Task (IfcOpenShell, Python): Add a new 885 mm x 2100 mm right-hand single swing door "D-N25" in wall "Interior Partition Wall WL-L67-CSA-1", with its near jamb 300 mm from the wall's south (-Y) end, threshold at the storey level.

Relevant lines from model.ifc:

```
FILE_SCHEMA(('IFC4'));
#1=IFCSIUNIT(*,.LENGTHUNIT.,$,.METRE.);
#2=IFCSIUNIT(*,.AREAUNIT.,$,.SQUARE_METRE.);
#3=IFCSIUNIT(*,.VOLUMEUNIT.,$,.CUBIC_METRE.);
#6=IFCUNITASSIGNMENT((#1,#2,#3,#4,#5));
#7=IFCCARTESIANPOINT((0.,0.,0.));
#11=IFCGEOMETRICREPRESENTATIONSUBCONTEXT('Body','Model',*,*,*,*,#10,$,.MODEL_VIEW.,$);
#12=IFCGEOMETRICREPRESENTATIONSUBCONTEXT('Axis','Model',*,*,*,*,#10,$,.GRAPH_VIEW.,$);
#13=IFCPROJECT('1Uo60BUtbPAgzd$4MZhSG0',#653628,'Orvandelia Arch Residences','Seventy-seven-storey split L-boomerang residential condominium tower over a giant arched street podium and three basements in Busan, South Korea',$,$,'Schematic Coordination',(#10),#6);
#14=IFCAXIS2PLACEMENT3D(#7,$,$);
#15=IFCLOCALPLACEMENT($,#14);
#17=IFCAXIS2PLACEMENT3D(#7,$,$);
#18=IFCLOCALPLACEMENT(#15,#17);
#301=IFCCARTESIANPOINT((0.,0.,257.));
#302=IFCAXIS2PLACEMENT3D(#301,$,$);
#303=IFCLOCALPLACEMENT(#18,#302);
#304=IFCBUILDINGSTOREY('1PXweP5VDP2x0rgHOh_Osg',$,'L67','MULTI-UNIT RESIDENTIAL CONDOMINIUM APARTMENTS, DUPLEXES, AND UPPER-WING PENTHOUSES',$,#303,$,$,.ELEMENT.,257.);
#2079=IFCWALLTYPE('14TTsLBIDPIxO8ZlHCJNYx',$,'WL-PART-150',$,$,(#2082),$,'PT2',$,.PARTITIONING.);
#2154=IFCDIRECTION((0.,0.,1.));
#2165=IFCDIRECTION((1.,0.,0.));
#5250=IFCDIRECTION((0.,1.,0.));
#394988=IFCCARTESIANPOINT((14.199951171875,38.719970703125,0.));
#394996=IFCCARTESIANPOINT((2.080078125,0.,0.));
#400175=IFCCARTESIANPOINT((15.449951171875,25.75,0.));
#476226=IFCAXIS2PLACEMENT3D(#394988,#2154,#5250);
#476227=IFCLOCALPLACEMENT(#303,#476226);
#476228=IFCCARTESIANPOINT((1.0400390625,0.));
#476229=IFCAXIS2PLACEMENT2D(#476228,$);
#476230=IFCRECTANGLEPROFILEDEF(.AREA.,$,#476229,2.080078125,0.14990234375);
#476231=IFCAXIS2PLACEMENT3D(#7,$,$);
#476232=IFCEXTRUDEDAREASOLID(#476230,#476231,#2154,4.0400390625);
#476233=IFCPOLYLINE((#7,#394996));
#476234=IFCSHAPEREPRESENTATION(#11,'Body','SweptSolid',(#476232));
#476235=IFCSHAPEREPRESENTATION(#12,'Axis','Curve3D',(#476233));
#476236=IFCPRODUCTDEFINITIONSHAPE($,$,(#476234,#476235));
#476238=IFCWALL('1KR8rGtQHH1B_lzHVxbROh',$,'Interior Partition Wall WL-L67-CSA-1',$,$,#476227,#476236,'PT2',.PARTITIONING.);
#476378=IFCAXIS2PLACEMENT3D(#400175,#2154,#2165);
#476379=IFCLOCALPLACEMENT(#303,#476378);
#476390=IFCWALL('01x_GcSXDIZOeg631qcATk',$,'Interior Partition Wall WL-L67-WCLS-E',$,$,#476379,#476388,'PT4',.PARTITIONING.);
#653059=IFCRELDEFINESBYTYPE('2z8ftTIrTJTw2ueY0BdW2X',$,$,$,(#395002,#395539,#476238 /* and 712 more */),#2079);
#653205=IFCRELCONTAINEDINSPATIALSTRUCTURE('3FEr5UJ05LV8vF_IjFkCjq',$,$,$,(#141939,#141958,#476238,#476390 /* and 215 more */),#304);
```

```python
import numpy as np
import ifcopenshell
import ifcopenshell.api.feature
import ifcopenshell.api.geometry
import ifcopenshell.api.root
import ifcopenshell.api.spatial
import ifcopenshell.geom
import ifcopenshell.util.element
import ifcopenshell.util.placement
import ifcopenshell.util.representation
import ifcopenshell.util.shape
import ifcopenshell.util.unit

model = ifcopenshell.open("model.ifc")
unit_scale = ifcopenshell.util.unit.calculate_unit_scale(model)
settings = ifcopenshell.geom.settings()


def volume(element):
    """Net volume in cubic metres, openings subtracted."""
    shape = ifcopenshell.geom.create_shape(settings, element)
    return ifcopenshell.util.shape.get_volume(shape.geometry)


wall = model.by_guid("1KR8rGtQHH1B_lzHVxbROh")
storey = ifcopenshell.util.element.get_container(wall, ifc_class="IfcBuildingStorey")
context = ifcopenshell.util.representation.get_context(model, "Model", "Body", "MODEL_VIEW")
before = volume(wall)

width, height, from_end, sill = 0.885, 2.1, 0.3, 0.0  # metres

# The wall runs along its own X axis, and the end named is its -X end.
wall_shape = ifcopenshell.geom.create_shape(settings, wall)
x, y, z = ifcopenshell.util.shape.get_vertices(wall_shape.geometry).T
start = x.min() + from_end
face, thickness = float(y.min()), float(y.max() - y.min())
wall_matrix = ifcopenshell.util.placement.get_local_placement(wall.ObjectPlacement)
level = ifcopenshell.util.placement.get_local_placement(storey.ObjectPlacement)[2, 3]


def in_wall(x, y):
    """Placement at x, y metres in the wall's axes, at sill height."""
    matrix = wall_matrix.copy()
    matrix[:, 3] = wall_matrix @ np.array([x / unit_scale, y / unit_scale, 0.0, 1.0])
    matrix[2, 3] = level + sill / unit_scale
    return matrix


# Opening: a box that overshoots both wall faces by 50 mm.
opening = ifcopenshell.api.root.create_entity(model, ifc_class="IfcOpeningElement", predefined_type="OPENING")
box = ifcopenshell.api.geometry.add_wall_representation(
    model, context=context, length=width, height=height, thickness=thickness + 0.1
)
ifcopenshell.api.geometry.assign_representation(model, product=opening, representation=box)
ifcopenshell.api.geometry.edit_object_placement(model, product=opening, matrix=in_wall(start, face - 0.05), is_si=False)
ifcopenshell.api.feature.add_feature(model, feature=opening, element=wall)

door = ifcopenshell.api.root.create_entity(model, ifc_class="IfcDoor", name="D-N25", predefined_type="DOOR")
door.OverallWidth, door.OverallHeight = width / unit_scale, height / unit_scale
door.OperationType = "SINGLE_SWING_RIGHT"
body = ifcopenshell.api.geometry.add_door_representation(
    model,
    context=context,
    overall_width=door.OverallWidth,
    overall_height=door.OverallHeight,
    operation_type="SINGLE_SWING_RIGHT",
    lining_properties={"LiningDepth": thickness / unit_scale, "ThresholdDepth": thickness / unit_scale},
)
ifcopenshell.api.geometry.assign_representation(model, product=door, representation=body)
ifcopenshell.api.spatial.assign_container(model, products=[door], relating_structure=storey)
ifcopenshell.api.feature.add_filling(model, opening=opening, element=door)

# The lining spans the wall, so the door starts at the wall face.
ifcopenshell.api.geometry.edit_object_placement(model, product=door, matrix=in_wall(start, face), is_si=False)

after = volume(wall)

print(f"wall volume {before:.3f} -> {after:.3f} m3")

model.write("model_edited.ifc")
```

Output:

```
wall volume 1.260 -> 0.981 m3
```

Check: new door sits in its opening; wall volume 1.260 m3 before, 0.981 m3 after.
